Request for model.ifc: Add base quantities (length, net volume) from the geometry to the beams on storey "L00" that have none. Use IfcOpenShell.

First a look at what the model holds.

```python
import ifcopenshell
import ifcopenshell.util.element
import ifcopenshell.util.unit

model = ifcopenshell.open("model.ifc")
print(model.schema)
for unit_type in ("LENGTHUNIT", "AREAUNIT", "VOLUMEUNIT"):
    print(unit_type, ifcopenshell.util.unit.calculate_unit_scale(model, unit_type))
storey = next(s for s in model.by_type("IfcBuildingStorey") if s.Name == "L00")
beams = [e for e in ifcopenshell.util.element.get_decomposition(storey) if e.is_a("IfcBeam")]
for e in sorted(beams, key=lambda e: e.id()):
    print(e.id(), e.is_a(), e.Name, list(ifcopenshell.util.element.get_psets(e, qtos_only=True)), sep=" | ")
```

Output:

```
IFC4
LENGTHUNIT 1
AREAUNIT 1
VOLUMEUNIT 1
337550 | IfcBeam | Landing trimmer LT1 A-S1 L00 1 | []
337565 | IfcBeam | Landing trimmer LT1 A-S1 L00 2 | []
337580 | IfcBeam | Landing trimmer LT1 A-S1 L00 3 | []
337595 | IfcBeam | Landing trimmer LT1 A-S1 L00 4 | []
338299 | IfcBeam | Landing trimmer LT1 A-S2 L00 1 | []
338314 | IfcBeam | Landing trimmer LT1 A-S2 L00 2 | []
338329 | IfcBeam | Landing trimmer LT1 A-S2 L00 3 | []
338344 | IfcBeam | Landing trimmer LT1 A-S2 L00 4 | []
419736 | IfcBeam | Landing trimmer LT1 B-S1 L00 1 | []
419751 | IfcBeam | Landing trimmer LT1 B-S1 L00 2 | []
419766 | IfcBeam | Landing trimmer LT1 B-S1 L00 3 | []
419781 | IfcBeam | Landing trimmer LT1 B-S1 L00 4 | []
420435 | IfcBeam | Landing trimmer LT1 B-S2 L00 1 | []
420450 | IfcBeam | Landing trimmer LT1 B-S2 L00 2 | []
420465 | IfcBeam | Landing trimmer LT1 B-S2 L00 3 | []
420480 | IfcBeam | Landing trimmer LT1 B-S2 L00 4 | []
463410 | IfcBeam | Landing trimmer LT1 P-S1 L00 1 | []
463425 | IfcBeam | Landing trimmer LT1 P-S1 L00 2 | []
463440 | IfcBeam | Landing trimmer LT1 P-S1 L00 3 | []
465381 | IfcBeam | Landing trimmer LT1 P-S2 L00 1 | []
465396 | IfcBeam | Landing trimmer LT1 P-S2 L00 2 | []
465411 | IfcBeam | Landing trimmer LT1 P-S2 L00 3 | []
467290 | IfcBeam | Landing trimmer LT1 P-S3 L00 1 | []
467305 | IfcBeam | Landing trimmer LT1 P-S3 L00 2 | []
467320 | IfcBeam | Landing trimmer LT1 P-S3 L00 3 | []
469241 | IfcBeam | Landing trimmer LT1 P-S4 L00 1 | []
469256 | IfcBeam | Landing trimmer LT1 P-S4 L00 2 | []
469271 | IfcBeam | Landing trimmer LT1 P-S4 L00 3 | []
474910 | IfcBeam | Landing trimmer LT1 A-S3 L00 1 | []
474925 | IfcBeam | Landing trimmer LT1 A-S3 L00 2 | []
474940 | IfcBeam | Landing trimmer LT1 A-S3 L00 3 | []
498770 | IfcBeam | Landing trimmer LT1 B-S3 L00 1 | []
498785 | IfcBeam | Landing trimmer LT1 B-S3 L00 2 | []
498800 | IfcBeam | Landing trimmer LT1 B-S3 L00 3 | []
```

```python
import ifcopenshell
import ifcopenshell.api.pset
import ifcopenshell.geom
import ifcopenshell.util.element
import ifcopenshell.util.shape
import ifcopenshell.util.unit

model = ifcopenshell.open("model.ifc")
unit_scale = ifcopenshell.util.unit.calculate_unit_scale(model)
volume_scale = ifcopenshell.util.unit.calculate_unit_scale(model, "VOLUMEUNIT")
settings = ifcopenshell.geom.settings()

storey = next(s for s in model.by_type("IfcBuildingStorey") if s.Name == "L00")
beams = [e for e in ifcopenshell.util.element.get_decomposition(storey) if e.is_a("IfcBeam")]

for e in sorted(beams, key=lambda e: e.id()):
    if ifcopenshell.util.element.get_psets(e, qtos_only=True, should_inherit=False):
        continue
    # Geometry comes back in metres, in the element's own axes.
    shape = ifcopenshell.geom.create_shape(settings, e)
    values = {
        "Length": ifcopenshell.util.shape.get_max_xyz(shape.geometry) / unit_scale,
        "NetVolume": ifcopenshell.util.shape.get_volume(shape.geometry) / volume_scale,
    }
    qto = ifcopenshell.api.pset.add_qto(model, product=e, name="Qto_BeamBaseQuantities")
    ifcopenshell.api.pset.edit_qto(model, qto=qto, properties=values)
    print(e.id(), {k: round(v, 3) for k, v in values.items()})

model.write("model_v2.ifc")
```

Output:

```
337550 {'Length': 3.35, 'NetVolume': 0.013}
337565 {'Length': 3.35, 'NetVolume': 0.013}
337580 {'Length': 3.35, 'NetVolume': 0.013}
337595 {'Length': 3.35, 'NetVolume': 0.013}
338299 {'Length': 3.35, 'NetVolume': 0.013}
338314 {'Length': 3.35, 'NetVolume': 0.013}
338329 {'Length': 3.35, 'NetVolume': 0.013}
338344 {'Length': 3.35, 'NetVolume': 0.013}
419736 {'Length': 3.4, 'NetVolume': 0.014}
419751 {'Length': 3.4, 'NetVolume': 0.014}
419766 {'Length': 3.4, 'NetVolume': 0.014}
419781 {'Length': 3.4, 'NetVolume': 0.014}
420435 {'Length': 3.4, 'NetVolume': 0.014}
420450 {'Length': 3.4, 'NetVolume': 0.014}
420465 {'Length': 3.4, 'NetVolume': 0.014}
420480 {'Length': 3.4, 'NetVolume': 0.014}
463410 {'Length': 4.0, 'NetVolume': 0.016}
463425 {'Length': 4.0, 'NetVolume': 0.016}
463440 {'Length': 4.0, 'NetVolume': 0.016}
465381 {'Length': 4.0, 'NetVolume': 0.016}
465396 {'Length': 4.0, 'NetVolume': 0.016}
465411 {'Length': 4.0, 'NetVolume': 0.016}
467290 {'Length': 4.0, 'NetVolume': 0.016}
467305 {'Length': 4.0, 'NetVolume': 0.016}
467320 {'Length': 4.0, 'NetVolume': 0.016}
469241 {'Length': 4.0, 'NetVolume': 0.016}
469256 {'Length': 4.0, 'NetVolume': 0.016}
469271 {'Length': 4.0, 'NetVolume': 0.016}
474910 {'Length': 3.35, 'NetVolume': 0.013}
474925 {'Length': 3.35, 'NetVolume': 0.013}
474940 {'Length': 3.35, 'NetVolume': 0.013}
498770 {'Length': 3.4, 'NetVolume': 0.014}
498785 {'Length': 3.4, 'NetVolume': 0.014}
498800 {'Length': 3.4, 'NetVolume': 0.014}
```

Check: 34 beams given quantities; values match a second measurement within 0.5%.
